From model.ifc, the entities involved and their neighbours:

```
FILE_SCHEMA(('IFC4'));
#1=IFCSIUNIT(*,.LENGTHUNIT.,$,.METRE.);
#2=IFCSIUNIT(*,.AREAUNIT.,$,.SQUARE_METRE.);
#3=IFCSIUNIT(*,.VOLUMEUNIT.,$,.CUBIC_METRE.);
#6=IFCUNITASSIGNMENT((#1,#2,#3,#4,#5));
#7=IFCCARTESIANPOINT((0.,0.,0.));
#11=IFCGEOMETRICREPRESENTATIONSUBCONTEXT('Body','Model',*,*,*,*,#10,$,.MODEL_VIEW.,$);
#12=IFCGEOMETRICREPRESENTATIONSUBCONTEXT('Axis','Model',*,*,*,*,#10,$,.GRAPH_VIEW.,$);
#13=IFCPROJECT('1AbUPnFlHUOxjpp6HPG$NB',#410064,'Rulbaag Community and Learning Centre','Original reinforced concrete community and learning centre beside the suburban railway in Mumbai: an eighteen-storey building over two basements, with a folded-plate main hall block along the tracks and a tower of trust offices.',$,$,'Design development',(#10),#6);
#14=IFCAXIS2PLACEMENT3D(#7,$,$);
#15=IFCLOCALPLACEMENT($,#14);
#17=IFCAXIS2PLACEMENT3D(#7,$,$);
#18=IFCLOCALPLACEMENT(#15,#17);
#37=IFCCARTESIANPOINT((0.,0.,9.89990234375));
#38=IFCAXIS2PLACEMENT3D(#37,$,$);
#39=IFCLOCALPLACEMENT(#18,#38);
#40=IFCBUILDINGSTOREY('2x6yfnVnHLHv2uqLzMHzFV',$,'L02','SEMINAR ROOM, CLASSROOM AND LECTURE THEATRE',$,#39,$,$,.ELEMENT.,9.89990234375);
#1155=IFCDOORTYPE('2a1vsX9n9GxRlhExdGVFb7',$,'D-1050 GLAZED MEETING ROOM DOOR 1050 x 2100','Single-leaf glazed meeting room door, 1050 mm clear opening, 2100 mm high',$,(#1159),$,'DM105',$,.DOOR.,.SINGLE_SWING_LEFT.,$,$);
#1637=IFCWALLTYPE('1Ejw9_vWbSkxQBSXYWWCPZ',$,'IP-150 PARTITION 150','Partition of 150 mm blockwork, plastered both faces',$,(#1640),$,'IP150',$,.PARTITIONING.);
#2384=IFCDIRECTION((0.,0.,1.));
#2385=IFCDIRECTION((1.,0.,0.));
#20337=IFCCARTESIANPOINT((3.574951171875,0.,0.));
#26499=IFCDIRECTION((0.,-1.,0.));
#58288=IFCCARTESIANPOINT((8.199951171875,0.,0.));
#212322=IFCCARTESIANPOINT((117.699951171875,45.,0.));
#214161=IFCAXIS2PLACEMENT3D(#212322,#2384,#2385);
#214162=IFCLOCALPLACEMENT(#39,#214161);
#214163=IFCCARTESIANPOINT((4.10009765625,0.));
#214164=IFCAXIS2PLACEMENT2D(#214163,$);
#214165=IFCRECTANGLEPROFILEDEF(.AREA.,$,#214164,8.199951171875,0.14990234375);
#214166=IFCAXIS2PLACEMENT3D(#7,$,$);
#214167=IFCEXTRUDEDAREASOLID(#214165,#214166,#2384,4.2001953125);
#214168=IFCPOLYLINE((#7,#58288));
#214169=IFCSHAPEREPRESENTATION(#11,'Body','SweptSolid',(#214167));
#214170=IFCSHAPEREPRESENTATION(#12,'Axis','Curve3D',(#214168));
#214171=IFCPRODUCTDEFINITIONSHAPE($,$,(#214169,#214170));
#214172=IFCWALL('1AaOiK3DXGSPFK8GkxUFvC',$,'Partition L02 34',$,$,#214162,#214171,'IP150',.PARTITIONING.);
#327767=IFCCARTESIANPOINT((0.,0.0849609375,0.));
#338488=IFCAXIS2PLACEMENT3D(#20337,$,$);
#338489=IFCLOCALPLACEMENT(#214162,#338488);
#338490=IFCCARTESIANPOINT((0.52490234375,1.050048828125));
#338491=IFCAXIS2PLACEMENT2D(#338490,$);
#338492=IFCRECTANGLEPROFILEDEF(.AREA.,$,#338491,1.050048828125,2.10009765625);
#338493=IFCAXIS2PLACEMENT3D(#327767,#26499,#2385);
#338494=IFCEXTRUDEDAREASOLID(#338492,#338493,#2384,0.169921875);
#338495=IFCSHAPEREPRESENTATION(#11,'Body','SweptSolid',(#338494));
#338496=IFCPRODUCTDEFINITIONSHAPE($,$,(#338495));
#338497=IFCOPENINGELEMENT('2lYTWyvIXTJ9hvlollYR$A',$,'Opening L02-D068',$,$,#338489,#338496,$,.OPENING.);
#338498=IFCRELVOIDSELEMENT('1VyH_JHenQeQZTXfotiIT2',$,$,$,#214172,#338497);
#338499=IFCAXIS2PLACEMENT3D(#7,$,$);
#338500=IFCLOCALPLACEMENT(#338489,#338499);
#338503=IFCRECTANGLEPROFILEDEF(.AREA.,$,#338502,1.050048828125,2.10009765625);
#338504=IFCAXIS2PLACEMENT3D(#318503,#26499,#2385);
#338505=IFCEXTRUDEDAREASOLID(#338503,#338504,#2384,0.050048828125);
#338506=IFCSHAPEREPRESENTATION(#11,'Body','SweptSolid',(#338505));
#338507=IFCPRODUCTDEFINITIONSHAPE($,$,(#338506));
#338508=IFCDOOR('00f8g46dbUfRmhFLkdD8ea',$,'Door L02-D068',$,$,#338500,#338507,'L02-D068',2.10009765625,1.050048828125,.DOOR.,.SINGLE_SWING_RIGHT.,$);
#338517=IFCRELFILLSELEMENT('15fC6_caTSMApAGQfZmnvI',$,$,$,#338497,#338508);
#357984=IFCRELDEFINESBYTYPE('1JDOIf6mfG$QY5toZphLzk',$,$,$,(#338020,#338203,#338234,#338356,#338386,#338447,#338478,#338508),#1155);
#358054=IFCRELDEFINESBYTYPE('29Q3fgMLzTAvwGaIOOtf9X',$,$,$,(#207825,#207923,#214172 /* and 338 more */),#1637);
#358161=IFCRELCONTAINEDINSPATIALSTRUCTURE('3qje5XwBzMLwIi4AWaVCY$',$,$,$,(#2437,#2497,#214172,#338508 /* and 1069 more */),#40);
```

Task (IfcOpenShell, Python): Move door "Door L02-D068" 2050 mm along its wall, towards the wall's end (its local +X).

```python
import ifcopenshell
import ifcopenshell.api.geometry
import ifcopenshell.util.placement
import ifcopenshell.util.unit

model = ifcopenshell.open("model.ifc")
unit_scale = ifcopenshell.util.unit.calculate_unit_scale(model)

door = model.by_guid("00f8g46dbUfRmhFLkdD8ea")
opening = door.FillsVoids[0].RelatingOpeningElement
wall = opening.VoidsElements[0].RelatingBuildingElement

wall_matrix = ifcopenshell.util.placement.get_local_placement(wall.ObjectPlacement)
shift = wall_matrix[:3, 0] * 2.05 / unit_scale
before = ifcopenshell.util.placement.get_local_placement(door.ObjectPlacement)[:3, 3].copy()

# The door is placed relative to its opening, so it follows when the opening moves.
matrix = ifcopenshell.util.placement.get_local_placement(opening.ObjectPlacement)
matrix[:3, 3] += shift
ifcopenshell.api.geometry.edit_object_placement(
    model, product=opening, matrix=matrix, is_si=False, should_transform_children=True
)

after = ifcopenshell.util.placement.get_local_placement(door.ObjectPlacement)[:3, 3]
print("door moved by", (after - before).round(3) + 0.0)

model.write("model-out.ifc")
```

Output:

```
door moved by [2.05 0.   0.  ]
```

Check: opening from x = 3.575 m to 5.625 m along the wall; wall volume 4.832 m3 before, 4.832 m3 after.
